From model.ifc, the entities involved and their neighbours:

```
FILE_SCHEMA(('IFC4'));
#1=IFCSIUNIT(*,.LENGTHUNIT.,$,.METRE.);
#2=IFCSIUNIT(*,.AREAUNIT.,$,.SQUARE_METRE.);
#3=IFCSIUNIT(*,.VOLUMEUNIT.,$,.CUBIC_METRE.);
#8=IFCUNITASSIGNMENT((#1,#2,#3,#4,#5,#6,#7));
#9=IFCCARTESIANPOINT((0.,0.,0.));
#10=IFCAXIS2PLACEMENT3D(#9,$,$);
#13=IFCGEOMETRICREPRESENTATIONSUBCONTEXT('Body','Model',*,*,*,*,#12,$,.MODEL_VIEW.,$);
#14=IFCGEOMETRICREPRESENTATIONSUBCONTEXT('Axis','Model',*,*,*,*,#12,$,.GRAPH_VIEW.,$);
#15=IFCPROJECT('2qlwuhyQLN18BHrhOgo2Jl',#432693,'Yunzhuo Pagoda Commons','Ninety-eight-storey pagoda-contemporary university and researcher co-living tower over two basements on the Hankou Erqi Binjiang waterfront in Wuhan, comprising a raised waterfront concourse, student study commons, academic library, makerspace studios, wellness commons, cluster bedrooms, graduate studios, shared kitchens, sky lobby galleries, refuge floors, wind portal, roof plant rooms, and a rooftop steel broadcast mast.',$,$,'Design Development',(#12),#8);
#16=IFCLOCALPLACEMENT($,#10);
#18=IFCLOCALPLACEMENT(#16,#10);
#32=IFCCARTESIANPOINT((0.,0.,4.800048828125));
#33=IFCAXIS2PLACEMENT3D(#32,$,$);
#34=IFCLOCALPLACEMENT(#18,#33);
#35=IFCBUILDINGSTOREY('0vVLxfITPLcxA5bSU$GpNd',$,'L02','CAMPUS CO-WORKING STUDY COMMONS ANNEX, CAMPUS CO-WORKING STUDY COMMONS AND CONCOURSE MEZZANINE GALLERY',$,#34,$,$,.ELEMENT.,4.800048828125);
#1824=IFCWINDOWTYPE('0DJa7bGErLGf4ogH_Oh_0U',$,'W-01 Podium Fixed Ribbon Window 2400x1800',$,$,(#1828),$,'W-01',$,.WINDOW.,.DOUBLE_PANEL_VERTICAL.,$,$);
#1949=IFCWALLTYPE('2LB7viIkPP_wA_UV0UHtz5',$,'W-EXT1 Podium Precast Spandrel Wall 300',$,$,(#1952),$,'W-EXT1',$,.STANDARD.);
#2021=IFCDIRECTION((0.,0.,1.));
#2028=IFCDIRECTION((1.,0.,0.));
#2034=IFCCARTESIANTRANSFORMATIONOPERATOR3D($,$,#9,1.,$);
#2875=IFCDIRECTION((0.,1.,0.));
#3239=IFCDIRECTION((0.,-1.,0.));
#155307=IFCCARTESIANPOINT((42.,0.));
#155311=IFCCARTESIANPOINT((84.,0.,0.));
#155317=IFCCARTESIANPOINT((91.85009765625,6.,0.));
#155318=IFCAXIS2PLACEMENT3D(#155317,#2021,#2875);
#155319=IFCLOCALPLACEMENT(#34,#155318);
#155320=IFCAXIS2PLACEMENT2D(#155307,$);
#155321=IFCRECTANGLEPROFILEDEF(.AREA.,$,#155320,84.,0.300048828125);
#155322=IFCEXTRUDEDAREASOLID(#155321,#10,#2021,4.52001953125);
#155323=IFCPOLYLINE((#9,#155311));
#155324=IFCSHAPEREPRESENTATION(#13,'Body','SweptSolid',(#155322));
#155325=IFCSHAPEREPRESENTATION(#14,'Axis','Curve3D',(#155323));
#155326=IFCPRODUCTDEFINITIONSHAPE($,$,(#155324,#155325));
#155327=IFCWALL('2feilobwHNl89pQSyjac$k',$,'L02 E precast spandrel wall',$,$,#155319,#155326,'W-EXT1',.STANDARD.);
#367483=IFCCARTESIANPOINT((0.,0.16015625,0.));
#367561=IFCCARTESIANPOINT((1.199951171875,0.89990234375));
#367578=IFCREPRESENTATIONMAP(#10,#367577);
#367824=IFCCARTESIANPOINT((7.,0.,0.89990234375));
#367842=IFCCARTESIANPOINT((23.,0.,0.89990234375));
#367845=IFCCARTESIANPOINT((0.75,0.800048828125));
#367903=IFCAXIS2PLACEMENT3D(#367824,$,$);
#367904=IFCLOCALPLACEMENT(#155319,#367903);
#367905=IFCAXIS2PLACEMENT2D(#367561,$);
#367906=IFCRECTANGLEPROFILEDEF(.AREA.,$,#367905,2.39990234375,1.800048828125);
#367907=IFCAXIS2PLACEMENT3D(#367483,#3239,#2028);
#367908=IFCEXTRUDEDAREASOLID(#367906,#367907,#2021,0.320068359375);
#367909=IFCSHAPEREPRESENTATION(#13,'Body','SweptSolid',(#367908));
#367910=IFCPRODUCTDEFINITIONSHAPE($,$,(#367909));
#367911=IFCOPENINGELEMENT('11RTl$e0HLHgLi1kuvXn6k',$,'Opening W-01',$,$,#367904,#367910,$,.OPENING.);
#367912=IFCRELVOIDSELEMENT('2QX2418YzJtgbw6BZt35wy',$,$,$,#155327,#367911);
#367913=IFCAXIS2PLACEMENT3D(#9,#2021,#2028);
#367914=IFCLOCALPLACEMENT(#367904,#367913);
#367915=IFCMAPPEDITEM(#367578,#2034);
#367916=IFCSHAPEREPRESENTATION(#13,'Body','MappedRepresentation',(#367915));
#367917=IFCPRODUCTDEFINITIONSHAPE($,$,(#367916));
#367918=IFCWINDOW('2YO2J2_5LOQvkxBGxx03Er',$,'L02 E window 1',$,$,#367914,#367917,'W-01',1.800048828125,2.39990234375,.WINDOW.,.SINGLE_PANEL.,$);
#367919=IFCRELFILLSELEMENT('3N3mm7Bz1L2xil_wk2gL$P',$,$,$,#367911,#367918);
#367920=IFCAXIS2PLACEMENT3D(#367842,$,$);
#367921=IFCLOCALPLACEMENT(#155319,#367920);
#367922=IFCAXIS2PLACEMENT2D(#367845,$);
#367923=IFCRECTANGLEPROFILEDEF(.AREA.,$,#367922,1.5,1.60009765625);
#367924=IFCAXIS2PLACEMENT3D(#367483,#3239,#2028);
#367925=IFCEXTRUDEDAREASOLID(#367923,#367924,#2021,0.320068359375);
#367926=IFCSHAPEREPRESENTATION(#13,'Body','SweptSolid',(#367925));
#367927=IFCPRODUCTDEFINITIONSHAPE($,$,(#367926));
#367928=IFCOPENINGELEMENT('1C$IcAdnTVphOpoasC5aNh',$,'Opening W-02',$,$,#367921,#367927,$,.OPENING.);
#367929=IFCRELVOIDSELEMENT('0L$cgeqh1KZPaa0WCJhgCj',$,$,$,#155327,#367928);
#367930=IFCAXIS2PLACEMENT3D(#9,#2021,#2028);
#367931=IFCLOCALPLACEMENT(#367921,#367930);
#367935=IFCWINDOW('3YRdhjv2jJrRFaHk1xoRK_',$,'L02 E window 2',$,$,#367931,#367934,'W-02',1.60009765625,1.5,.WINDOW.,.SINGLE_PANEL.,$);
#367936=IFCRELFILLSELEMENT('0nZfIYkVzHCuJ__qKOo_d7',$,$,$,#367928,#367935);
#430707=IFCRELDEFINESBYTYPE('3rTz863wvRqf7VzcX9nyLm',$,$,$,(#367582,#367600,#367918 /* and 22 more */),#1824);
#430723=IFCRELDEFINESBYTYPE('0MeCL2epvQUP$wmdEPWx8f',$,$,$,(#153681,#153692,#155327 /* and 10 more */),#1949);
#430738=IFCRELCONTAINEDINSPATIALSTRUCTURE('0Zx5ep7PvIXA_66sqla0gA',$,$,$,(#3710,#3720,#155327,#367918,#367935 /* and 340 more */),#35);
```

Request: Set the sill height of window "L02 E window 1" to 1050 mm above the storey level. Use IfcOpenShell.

```python
import numpy as np
import ifcopenshell
import ifcopenshell.api.geometry
import ifcopenshell.geom
import ifcopenshell.util.element
import ifcopenshell.util.placement
import ifcopenshell.util.shape
import ifcopenshell.util.unit

model = ifcopenshell.open("model.ifc")
unit_scale = ifcopenshell.util.unit.calculate_unit_scale(model)

window = model.by_guid("2YO2J2_5LOQvkxBGxx03Er")
opening = window.FillsVoids[0].RelatingOpeningElement
storey = ifcopenshell.util.element.get_container(window, ifc_class="IfcBuildingStorey")
level = ifcopenshell.util.placement.get_local_placement(storey.ObjectPlacement)[2, 3]

# The opening's origin need not be at the sill, so measure its lowest point.
shape = ifcopenshell.geom.create_shape(ifcopenshell.geom.settings(), opening)
bottom = ifcopenshell.util.shape.get_shape_bottom_elevation(shape, shape.geometry) / unit_scale
dz = level + 1.05 - bottom

shift = np.array([0.0, 0.0, dz])
# The window is placed relative to its opening, so it follows when the opening moves.
matrix = ifcopenshell.util.placement.get_local_placement(opening.ObjectPlacement)
matrix[:3, 3] += shift
ifcopenshell.api.geometry.edit_object_placement(
    model, product=opening, matrix=matrix, is_si=False, should_transform_children=True
)

print(f"moved by {dz * unit_scale:+.3f} m")

model.write("model_updated.ifc")
```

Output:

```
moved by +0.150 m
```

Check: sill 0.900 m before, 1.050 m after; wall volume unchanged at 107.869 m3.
